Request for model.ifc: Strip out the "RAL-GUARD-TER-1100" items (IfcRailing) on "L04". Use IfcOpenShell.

First a look at what the model holds.

```python
import ifcopenshell
import ifcopenshell.util.element

model = ifcopenshell.open("model.ifc")
print(model.schema)
storey = next(s for s in model.by_type("IfcBuildingStorey") if s.Name == "L04")
railings = [e for e in ifcopenshell.util.element.get_decomposition(storey) if e.is_a("IfcRailing")]
seen = {}
for e in railings:
    element_type = ifcopenshell.util.element.get_type(e)
    name = element_type.Name if element_type not in (None, e) else None
    seen[name] = seen.get(name, 0) + 1
for name, count in sorted(seen.items(), key=str):
    print(count, "x", name)
```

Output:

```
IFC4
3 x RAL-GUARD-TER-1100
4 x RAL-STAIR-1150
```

```python
import ifcopenshell
import ifcopenshell.api.root
import ifcopenshell.util.element

model = ifcopenshell.open("model.ifc")

storey = next(s for s in model.by_type("IfcBuildingStorey") if s.Name == "L04")
railings = [e for e in ifcopenshell.util.element.get_decomposition(storey) if e.is_a("IfcRailing")]
targets = [e for e in railings if (t := ifcopenshell.util.element.get_type(e)) not in (None, e) and t.Name == "RAL-GUARD-TER-1100"]

for e in targets:
    ifcopenshell.api.root.remove_product(model, product=e)
print(len(targets), "removed")

model.write("model_edited.ifc")
```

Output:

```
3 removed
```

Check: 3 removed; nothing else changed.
